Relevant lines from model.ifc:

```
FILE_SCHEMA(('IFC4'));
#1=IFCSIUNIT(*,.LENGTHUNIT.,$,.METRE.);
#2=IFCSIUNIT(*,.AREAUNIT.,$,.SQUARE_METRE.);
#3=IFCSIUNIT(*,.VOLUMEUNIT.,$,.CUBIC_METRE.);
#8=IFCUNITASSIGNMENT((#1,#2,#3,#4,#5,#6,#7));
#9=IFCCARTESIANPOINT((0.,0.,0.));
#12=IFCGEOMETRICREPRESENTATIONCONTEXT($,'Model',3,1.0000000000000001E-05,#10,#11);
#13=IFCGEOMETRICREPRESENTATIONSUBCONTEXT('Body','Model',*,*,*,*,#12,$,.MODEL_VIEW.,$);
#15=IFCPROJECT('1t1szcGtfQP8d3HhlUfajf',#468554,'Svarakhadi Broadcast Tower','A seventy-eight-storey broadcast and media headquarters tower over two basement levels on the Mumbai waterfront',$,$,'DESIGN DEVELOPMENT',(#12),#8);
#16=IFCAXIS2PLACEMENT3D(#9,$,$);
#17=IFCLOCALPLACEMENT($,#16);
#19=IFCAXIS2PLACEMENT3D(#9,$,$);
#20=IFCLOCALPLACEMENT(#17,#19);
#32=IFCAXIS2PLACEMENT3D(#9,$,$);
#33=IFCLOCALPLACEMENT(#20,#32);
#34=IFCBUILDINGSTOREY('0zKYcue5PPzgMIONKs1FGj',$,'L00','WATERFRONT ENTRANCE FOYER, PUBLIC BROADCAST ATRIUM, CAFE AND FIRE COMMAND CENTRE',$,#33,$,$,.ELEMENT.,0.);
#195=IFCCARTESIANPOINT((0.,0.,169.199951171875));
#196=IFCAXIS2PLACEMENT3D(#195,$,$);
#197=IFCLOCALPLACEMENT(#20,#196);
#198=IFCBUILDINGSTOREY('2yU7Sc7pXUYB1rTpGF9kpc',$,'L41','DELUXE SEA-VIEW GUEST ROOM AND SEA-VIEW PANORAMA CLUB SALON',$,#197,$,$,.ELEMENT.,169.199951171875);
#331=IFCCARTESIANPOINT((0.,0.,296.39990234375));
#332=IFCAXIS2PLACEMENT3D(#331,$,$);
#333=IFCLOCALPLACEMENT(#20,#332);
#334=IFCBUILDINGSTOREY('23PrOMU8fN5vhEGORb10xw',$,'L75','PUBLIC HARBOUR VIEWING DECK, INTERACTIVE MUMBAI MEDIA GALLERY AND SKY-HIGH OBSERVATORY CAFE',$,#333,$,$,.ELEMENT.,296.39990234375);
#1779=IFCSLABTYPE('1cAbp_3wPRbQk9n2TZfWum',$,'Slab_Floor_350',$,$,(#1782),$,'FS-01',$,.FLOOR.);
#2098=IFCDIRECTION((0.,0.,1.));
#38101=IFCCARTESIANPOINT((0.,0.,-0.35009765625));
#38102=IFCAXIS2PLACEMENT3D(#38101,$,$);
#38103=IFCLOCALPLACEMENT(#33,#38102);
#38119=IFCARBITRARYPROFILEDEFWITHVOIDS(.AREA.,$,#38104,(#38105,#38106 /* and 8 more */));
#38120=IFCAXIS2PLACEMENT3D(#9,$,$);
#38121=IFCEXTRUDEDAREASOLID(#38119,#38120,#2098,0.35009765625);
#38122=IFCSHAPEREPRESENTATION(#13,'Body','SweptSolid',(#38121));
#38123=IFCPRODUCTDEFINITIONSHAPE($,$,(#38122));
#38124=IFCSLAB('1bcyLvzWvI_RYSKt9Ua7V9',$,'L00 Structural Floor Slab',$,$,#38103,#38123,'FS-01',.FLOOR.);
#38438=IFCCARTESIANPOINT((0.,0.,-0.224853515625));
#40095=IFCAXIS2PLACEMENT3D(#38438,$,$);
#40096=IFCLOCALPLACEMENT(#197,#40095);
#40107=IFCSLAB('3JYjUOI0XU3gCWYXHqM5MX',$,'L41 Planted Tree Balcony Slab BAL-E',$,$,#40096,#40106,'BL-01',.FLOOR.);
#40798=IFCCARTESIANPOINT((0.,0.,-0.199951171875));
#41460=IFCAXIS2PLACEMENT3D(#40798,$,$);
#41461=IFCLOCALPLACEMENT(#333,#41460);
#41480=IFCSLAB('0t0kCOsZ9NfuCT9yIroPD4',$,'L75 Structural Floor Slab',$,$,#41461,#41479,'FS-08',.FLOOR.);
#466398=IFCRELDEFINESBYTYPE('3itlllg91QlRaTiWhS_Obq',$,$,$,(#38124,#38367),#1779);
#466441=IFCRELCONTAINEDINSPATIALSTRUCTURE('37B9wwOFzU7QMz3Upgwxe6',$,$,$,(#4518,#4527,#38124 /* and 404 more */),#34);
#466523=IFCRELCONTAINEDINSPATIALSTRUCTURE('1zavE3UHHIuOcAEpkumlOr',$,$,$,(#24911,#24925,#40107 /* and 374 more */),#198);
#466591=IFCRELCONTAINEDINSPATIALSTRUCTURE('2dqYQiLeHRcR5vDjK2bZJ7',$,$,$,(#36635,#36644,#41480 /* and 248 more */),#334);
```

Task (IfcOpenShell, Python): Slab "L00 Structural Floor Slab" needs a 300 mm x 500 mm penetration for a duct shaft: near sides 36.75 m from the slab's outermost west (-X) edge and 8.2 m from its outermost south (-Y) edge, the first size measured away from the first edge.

```python
import numpy as np
import ifcopenshell
import ifcopenshell.api.feature
import ifcopenshell.api.geometry
import ifcopenshell.api.root
import ifcopenshell.geom
import ifcopenshell.util.placement
import ifcopenshell.util.representation
import ifcopenshell.util.shape
import ifcopenshell.util.unit

model = ifcopenshell.open("model.ifc")
unit_scale = ifcopenshell.util.unit.calculate_unit_scale(model)
settings = ifcopenshell.geom.settings()


def volume(element):
    """Net volume in cubic metres, openings subtracted."""
    shape = ifcopenshell.geom.create_shape(settings, element)
    return ifcopenshell.util.shape.get_volume(shape.geometry)


slab = model.by_id(38124)
before = volume(slab)

# Extent in the slab's own axes, in metres. The edges named are its -X and -Y sides.
slab_shape = ifcopenshell.geom.create_shape(settings, slab)
vertices = ifcopenshell.util.shape.get_vertices(slab_shape.geometry)
x_min, y_min, bottom = vertices.min(axis=0)
top = vertices[:, 2].max()

opening = ifcopenshell.api.root.create_entity(model, ifc_class="IfcOpeningElement", name="Duct shaft opening", predefined_type="OPENING")
context = ifcopenshell.util.representation.get_context(model, "Model", "Body", "MODEL_VIEW")
width, depth = 0.3, 0.5
outline = [(0.0, 0.0), (width, 0.0), (width, depth), (0.0, depth), (0.0, 0.0)]
# Overshoot both faces by 50 mm so the cut is clean.
shape = ifcopenshell.api.geometry.add_slab_representation(
    model, context=context, depth=top - bottom + 0.1, polyline=outline
)
ifcopenshell.api.geometry.assign_representation(model, product=opening, representation=shape)

matrix = ifcopenshell.util.placement.get_local_placement(slab.ObjectPlacement)
matrix[:, 3] = matrix @ np.append(np.array([x_min + 36.75, y_min + 8.2, bottom - 0.05]) / unit_scale, 1.0)
ifcopenshell.api.geometry.edit_object_placement(model, product=opening, matrix=matrix, is_si=False)
ifcopenshell.api.feature.add_feature(model, feature=opening, element=slab)

after = volume(slab)

print(f"slab volume {before:.3f} -> {after:.3f} m3")

model.write("model-out.ifc")
```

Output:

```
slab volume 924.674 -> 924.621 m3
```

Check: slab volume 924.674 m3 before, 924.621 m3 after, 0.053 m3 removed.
